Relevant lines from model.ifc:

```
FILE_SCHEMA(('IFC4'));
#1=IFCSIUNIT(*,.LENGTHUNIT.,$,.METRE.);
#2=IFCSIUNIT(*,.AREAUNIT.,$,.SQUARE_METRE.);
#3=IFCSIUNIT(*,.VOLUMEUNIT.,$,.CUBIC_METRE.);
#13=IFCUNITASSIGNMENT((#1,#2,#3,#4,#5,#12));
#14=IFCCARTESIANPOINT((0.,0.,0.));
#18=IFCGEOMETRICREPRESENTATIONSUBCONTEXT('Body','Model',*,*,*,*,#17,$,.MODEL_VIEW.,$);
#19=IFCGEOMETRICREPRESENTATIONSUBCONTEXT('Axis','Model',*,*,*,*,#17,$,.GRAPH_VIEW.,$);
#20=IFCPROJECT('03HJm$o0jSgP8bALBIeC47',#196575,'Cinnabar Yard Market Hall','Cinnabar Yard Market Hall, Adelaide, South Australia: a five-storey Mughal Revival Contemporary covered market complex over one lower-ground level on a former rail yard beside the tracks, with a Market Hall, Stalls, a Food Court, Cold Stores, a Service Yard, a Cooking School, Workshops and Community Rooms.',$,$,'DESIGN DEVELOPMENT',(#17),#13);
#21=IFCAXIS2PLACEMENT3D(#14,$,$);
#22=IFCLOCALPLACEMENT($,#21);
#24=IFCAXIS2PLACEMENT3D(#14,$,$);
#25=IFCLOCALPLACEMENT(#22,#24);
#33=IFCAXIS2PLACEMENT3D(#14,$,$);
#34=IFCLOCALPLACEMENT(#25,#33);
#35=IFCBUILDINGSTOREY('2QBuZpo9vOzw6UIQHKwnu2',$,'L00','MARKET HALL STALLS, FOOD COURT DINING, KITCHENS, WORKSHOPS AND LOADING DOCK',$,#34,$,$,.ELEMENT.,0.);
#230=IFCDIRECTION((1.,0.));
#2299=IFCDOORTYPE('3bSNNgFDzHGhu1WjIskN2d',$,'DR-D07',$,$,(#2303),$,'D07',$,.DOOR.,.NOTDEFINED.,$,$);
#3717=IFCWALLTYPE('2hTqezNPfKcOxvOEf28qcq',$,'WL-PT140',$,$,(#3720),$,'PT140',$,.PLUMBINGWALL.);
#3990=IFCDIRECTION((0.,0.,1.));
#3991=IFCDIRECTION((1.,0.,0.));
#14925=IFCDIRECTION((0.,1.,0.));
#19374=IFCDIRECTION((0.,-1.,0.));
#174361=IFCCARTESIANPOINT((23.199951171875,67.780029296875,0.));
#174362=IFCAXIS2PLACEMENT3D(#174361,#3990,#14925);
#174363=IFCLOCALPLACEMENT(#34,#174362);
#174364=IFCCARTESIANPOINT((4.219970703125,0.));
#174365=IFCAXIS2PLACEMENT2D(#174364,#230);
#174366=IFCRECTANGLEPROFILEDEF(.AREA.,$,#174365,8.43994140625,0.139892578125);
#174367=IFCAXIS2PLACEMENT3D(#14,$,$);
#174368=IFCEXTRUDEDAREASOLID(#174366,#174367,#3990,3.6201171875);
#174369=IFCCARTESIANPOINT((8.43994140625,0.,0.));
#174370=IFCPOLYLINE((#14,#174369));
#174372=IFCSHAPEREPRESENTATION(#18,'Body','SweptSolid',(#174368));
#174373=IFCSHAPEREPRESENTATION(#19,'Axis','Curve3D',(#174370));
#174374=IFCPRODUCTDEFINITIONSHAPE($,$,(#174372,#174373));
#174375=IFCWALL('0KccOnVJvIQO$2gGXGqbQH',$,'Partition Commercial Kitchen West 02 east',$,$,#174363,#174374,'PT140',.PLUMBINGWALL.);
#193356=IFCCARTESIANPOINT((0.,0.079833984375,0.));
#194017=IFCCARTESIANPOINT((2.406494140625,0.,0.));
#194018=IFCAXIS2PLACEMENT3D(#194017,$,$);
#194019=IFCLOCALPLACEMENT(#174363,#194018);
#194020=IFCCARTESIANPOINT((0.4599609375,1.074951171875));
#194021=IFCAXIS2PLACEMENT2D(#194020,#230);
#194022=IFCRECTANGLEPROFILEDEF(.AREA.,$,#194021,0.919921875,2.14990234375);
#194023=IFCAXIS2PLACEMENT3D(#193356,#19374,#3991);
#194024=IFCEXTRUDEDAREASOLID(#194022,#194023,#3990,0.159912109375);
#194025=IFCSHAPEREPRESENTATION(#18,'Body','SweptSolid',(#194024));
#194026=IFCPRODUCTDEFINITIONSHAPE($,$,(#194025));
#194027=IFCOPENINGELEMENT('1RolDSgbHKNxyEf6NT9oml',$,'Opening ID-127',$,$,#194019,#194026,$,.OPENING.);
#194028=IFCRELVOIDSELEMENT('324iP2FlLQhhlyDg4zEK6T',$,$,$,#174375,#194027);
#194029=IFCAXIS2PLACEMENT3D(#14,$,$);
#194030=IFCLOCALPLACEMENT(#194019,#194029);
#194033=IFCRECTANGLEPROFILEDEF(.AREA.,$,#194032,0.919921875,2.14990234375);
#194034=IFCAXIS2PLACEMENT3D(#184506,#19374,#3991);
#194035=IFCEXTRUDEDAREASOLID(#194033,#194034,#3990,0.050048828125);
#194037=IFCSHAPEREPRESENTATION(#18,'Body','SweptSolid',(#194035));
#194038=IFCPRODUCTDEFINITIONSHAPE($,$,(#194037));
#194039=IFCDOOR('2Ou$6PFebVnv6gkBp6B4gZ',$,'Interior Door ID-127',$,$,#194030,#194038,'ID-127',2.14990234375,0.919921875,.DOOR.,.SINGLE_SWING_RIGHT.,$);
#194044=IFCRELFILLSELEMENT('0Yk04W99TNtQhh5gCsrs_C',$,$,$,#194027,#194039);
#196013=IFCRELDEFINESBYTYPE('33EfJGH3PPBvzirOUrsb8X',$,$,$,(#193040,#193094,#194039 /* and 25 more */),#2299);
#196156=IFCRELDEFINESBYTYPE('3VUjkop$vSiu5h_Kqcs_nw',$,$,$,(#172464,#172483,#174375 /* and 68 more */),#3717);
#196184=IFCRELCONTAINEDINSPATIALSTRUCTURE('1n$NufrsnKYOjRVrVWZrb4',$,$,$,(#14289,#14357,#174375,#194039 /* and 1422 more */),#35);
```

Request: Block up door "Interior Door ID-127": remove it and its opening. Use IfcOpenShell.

```python
import ifcopenshell
import ifcopenshell.api.feature
import ifcopenshell.api.root
import ifcopenshell.geom
import ifcopenshell.util.shape

model = ifcopenshell.open("model.ifc")
settings = ifcopenshell.geom.settings()


def volume(element):
    """Net volume in cubic metres, openings subtracted."""
    shape = ifcopenshell.geom.create_shape(settings, element)
    return ifcopenshell.util.shape.get_volume(shape.geometry)


door = model.by_id(194039)
opening = door.FillsVoids[0].RelatingOpeningElement
wall = opening.VoidsElements[0].RelatingBuildingElement
before = volume(wall)

ifcopenshell.api.root.remove_product(model, product=door)
ifcopenshell.api.feature.remove_feature(model, feature=opening)

after = volume(wall)

print(f"wall volume {before:.3f} -> {after:.3f} m3")

model.write("model_edited.ifc")
```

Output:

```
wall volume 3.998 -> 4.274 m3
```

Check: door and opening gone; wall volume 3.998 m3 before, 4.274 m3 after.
